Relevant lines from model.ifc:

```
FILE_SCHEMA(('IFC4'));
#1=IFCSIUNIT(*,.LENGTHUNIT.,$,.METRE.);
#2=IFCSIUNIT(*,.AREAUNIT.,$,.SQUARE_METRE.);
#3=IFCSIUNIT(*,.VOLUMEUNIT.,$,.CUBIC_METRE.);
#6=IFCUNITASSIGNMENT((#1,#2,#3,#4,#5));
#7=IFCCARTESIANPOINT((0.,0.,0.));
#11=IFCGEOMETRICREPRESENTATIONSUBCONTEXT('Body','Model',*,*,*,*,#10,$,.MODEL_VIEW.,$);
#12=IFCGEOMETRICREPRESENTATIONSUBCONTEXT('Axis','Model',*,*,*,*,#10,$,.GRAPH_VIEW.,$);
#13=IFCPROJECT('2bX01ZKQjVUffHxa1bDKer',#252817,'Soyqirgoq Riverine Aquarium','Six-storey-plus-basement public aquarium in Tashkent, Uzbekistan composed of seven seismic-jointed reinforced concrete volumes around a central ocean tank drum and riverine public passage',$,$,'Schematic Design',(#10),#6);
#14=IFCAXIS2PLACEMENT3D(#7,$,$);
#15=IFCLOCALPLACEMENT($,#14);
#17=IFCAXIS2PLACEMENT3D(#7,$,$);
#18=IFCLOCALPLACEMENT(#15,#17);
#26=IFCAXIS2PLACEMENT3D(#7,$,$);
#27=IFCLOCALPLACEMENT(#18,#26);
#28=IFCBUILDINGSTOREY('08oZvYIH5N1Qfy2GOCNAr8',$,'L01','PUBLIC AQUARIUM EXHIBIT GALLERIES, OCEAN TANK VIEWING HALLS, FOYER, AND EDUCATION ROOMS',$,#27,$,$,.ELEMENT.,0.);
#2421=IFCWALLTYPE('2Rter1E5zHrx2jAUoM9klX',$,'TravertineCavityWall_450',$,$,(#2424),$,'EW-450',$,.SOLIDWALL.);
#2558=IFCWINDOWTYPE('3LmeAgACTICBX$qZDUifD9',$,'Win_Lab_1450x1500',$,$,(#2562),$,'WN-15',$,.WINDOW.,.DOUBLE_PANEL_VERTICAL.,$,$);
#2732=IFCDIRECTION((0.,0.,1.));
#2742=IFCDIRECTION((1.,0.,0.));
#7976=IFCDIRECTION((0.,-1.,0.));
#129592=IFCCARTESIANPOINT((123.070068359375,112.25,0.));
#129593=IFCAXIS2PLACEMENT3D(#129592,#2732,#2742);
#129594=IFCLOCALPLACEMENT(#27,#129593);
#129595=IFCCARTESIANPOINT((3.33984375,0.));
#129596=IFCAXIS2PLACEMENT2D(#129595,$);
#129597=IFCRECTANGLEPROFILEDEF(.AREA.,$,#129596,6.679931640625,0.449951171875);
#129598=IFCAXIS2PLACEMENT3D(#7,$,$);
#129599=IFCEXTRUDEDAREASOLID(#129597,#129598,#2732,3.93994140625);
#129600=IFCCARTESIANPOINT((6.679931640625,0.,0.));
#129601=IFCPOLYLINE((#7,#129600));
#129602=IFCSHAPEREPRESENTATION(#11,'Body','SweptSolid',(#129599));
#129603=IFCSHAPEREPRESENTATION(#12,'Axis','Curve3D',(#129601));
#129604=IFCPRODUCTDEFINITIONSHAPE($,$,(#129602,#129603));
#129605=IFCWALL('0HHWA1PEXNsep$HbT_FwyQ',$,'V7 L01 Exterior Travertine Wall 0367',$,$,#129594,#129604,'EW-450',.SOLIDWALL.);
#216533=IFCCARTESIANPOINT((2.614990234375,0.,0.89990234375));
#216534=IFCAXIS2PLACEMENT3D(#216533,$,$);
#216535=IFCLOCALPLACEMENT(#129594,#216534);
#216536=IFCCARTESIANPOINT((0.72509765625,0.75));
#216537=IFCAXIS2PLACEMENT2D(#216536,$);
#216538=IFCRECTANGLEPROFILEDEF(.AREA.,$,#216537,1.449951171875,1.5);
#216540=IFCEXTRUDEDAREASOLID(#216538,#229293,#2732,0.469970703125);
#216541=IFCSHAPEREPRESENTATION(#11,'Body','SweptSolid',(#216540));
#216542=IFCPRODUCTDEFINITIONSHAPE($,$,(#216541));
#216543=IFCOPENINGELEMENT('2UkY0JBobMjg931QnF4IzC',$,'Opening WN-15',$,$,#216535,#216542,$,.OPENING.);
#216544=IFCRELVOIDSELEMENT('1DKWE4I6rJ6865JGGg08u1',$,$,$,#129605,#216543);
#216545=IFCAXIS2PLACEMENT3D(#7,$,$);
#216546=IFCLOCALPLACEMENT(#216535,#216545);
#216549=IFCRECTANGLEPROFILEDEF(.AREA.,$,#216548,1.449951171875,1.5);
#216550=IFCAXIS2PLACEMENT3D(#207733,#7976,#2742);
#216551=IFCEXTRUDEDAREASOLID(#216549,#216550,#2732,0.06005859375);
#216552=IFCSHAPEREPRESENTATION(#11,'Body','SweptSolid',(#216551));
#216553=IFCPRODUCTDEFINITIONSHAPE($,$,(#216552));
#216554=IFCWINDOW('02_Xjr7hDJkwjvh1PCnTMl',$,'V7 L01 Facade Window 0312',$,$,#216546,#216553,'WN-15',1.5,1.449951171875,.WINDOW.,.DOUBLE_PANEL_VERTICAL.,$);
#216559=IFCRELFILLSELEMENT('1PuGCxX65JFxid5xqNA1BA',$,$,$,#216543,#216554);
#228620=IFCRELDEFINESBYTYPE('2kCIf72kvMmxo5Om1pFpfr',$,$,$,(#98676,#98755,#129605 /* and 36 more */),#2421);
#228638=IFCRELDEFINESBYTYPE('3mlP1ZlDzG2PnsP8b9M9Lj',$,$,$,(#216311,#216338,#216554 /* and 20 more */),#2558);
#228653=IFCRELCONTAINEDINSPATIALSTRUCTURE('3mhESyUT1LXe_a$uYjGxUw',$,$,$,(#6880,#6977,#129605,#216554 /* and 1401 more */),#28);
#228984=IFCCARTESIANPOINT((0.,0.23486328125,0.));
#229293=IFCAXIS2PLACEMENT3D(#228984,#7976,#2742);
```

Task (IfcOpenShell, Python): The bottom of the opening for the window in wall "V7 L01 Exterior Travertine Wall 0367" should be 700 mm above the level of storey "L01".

```python
import numpy as np
import ifcopenshell
import ifcopenshell.api.geometry
import ifcopenshell.geom
import ifcopenshell.util.element
import ifcopenshell.util.placement
import ifcopenshell.util.shape
import ifcopenshell.util.unit

model = ifcopenshell.open("model.ifc")
unit_scale = ifcopenshell.util.unit.calculate_unit_scale(model)

window = model.by_id(216554)
opening = window.FillsVoids[0].RelatingOpeningElement
storey = ifcopenshell.util.element.get_container(window, ifc_class="IfcBuildingStorey")
level = ifcopenshell.util.placement.get_local_placement(storey.ObjectPlacement)[2, 3]

# The opening's origin need not be at the sill, so measure its lowest point.
shape = ifcopenshell.geom.create_shape(ifcopenshell.geom.settings(), opening)
bottom = ifcopenshell.util.shape.get_shape_bottom_elevation(shape, shape.geometry) / unit_scale
dz = level + 0.7 / unit_scale - bottom

shift = np.array([0.0, 0.0, dz])
# The window is placed relative to its opening, so it follows when the opening moves.
matrix = ifcopenshell.util.placement.get_local_placement(opening.ObjectPlacement)
matrix[:3, 3] += shift
ifcopenshell.api.geometry.edit_object_placement(
    model, product=opening, matrix=matrix, is_si=False, should_transform_children=True
)

print(f"moved by {dz * unit_scale:+.3f} m")

model.write("model_rev.ifc")
```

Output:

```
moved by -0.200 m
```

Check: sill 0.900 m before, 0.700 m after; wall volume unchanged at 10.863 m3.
